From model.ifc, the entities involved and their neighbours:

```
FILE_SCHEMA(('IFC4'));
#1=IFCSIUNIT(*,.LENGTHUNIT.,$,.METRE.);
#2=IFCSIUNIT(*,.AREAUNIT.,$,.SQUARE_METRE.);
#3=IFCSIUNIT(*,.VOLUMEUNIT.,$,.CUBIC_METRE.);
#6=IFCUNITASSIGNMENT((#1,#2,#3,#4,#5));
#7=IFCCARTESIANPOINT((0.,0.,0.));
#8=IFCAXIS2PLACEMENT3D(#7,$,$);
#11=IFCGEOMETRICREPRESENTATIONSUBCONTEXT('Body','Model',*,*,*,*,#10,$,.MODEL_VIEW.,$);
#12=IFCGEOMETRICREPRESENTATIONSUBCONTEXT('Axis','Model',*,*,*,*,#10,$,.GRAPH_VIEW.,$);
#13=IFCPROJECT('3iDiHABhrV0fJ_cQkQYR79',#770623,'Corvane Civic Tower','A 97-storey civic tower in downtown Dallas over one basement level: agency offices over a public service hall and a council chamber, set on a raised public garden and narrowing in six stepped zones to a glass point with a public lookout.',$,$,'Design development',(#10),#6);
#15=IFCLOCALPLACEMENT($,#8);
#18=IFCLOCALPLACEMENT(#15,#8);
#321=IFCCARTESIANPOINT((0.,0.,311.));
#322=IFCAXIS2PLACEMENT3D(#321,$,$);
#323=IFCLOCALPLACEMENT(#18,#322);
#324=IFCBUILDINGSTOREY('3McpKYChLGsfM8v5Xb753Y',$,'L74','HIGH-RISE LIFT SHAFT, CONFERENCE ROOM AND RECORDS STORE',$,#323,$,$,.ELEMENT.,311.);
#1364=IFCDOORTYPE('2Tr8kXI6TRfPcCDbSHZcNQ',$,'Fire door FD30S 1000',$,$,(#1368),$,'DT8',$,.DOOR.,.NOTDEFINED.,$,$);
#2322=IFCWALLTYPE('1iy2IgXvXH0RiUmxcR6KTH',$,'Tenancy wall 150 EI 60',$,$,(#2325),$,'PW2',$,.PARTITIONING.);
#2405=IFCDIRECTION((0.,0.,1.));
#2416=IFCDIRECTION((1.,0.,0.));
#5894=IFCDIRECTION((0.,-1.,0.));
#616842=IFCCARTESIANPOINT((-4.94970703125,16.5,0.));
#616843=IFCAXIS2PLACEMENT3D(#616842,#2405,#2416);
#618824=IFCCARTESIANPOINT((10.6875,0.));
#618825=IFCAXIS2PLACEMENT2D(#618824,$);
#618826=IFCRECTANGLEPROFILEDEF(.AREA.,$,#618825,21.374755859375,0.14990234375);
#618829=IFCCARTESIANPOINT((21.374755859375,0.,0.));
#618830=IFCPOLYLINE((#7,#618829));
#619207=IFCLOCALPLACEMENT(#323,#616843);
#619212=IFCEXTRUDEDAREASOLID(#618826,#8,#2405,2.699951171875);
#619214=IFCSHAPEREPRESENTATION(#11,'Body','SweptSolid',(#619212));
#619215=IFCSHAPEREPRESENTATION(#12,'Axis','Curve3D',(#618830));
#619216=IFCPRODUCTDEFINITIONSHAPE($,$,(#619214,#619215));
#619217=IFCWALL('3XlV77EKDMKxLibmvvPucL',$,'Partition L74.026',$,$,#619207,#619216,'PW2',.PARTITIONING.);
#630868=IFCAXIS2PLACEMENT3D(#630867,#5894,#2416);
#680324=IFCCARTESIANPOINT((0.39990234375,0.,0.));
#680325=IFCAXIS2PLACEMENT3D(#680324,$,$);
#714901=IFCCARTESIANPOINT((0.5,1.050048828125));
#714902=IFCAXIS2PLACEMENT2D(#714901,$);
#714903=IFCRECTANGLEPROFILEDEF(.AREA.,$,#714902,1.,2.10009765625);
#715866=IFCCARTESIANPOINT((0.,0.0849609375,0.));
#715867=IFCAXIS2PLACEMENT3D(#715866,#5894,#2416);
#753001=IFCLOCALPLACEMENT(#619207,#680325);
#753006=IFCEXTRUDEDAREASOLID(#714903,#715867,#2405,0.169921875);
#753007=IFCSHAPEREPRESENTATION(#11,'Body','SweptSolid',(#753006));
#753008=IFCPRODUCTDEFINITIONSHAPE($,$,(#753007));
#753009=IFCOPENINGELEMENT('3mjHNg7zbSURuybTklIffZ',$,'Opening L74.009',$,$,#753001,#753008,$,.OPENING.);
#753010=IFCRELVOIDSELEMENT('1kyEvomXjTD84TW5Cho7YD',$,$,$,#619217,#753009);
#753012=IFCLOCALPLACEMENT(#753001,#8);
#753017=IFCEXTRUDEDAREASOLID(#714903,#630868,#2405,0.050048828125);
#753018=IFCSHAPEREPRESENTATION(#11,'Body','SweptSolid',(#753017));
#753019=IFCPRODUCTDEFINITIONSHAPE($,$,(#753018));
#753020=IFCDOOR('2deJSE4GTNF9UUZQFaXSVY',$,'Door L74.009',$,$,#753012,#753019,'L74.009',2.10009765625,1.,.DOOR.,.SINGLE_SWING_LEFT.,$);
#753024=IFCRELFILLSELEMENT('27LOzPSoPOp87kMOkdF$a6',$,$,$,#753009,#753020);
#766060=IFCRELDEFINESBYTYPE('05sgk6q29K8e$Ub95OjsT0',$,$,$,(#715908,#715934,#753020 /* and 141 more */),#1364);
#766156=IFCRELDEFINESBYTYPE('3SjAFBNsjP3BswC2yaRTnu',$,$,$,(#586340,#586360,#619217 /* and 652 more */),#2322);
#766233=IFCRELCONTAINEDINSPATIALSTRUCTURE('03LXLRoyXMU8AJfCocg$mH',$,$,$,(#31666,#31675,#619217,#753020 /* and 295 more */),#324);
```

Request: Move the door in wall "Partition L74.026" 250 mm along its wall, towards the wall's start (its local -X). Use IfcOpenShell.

```python
import ifcopenshell
import ifcopenshell.api.geometry
import ifcopenshell.util.placement

model = ifcopenshell.open("model.ifc")

door = model.by_guid("2deJSE4GTNF9UUZQFaXSVY")
opening = door.FillsVoids[0].RelatingOpeningElement
wall = opening.VoidsElements[0].RelatingBuildingElement

wall_matrix = ifcopenshell.util.placement.get_local_placement(wall.ObjectPlacement)
shift = wall_matrix[:3, 0] * -0.25
before = ifcopenshell.util.placement.get_local_placement(door.ObjectPlacement)[:3, 3].copy()

# The door is placed relative to its opening, so it follows when the opening moves.
matrix = ifcopenshell.util.placement.get_local_placement(opening.ObjectPlacement)
matrix[:3, 3] += shift
ifcopenshell.api.geometry.edit_object_placement(
    model, product=opening, matrix=matrix, is_si=False, should_transform_children=True
)

after = ifcopenshell.util.placement.get_local_placement(door.ObjectPlacement)[:3, 3]
print("door moved by", (after - before).round(3) + 0.0)

model.write("model_rev.ifc")
```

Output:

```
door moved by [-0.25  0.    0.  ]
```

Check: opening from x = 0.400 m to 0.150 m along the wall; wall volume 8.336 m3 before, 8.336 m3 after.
